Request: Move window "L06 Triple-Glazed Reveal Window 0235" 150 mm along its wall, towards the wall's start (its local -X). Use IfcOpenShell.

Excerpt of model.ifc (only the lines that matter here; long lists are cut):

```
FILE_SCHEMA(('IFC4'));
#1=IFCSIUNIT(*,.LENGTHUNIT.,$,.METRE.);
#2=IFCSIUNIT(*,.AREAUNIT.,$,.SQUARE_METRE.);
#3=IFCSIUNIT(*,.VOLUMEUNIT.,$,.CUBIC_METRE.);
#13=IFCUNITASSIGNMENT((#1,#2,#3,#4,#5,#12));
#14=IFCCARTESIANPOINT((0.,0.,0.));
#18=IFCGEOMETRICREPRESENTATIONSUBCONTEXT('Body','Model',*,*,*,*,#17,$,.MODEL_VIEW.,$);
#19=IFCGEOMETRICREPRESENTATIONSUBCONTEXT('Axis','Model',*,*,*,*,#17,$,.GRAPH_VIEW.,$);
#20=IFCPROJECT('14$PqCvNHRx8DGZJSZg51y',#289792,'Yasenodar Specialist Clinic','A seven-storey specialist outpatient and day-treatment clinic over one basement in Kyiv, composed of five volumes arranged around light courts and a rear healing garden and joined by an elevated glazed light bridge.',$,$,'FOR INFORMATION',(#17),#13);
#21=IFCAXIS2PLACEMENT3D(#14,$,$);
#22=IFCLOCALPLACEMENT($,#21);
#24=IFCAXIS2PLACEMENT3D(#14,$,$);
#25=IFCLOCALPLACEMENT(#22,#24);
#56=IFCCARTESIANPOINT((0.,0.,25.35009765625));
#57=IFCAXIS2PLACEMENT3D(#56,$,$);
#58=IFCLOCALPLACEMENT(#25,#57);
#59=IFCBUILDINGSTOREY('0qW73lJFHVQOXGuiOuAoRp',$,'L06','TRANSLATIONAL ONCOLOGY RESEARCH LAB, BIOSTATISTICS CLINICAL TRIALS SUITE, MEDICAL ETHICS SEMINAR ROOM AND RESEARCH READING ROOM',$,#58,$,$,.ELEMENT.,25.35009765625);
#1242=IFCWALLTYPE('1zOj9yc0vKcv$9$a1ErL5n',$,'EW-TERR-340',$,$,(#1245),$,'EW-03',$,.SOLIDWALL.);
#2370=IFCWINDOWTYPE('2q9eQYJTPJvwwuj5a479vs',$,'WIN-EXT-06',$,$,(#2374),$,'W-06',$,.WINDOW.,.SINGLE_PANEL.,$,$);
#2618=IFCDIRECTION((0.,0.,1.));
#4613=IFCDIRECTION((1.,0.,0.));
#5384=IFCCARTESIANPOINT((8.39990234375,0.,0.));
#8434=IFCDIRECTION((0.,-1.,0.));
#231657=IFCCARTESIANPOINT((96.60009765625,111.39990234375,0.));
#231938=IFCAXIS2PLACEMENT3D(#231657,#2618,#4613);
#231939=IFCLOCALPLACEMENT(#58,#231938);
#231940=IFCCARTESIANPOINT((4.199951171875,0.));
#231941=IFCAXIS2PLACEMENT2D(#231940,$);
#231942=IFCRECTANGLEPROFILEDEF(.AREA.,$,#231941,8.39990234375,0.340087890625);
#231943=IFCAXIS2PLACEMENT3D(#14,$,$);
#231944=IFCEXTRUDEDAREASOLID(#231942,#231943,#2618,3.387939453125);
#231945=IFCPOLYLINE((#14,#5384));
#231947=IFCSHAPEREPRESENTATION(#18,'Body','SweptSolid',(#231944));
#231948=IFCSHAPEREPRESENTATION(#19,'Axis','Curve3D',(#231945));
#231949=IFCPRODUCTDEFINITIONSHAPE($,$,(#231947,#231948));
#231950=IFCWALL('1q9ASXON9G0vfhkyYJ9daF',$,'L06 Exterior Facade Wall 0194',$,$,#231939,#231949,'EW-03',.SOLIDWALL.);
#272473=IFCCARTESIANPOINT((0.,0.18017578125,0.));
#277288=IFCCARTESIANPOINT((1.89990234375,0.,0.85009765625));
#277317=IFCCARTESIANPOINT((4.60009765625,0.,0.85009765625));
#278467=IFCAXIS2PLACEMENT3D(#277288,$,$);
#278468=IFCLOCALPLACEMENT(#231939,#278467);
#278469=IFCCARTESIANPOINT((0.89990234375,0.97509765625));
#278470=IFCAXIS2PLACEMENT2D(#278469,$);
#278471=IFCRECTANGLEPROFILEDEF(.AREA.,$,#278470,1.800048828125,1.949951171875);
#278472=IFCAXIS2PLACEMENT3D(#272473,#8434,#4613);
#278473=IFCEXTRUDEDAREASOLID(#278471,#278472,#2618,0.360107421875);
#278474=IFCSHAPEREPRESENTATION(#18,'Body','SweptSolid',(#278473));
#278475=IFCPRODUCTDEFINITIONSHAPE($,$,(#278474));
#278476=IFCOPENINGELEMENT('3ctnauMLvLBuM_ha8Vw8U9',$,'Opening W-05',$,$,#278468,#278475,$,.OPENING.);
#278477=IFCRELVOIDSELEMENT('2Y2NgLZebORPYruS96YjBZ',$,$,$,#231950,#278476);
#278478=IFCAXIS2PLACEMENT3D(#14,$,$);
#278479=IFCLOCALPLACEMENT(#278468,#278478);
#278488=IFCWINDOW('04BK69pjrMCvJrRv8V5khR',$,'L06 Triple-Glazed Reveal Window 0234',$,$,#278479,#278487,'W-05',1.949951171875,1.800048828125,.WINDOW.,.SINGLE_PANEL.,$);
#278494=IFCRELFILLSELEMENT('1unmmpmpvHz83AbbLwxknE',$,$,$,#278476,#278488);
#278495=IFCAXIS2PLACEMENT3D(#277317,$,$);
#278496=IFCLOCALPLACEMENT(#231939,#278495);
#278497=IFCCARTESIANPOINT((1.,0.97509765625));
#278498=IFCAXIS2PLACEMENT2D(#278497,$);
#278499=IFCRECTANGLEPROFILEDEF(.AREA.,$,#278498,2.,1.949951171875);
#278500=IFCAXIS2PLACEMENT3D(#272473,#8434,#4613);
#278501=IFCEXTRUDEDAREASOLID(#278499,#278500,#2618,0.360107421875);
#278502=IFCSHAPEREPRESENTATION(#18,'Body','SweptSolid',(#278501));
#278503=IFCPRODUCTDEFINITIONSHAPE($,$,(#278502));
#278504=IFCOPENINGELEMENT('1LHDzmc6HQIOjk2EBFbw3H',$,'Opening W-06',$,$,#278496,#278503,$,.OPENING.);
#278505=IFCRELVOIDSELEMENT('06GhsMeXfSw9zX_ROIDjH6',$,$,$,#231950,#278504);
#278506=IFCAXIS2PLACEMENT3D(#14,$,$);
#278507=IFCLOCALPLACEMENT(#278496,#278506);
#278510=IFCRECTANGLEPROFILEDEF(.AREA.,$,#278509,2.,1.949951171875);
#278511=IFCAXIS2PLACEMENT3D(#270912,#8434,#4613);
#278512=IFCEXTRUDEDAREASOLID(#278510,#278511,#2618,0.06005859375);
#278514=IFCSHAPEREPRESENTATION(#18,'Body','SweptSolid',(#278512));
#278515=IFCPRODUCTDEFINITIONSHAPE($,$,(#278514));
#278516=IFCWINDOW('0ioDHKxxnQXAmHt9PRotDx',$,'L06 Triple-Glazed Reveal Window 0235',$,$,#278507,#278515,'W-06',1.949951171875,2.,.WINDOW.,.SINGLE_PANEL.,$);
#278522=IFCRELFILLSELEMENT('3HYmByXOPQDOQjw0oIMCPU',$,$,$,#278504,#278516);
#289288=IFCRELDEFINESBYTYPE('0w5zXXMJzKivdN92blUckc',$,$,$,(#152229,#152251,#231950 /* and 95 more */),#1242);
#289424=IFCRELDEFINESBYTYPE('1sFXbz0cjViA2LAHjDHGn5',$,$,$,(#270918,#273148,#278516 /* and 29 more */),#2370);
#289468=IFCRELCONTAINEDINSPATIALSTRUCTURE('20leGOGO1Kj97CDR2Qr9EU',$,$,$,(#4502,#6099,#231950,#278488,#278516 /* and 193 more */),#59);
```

```python
import ifcopenshell
import ifcopenshell.api.geometry
import ifcopenshell.util.placement

model = ifcopenshell.open("model.ifc")

window = model.by_id(278516)
opening = window.FillsVoids[0].RelatingOpeningElement
wall = opening.VoidsElements[0].RelatingBuildingElement

wall_matrix = ifcopenshell.util.placement.get_local_placement(wall.ObjectPlacement)
shift = wall_matrix[:3, 0] * -0.15
before = ifcopenshell.util.placement.get_local_placement(window.ObjectPlacement)[:3, 3].copy()

# The window is placed relative to its opening, so it follows when the opening moves.
matrix = ifcopenshell.util.placement.get_local_placement(opening.ObjectPlacement)
matrix[:3, 3] += shift
ifcopenshell.api.geometry.edit_object_placement(
    model, product=opening, matrix=matrix, is_si=False, should_transform_children=True
)

after = ifcopenshell.util.placement.get_local_placement(window.ObjectPlacement)[:3, 3]
print("window moved by", (after - before).round(3) + 0.0)

model.write("model_v2.ifc")
```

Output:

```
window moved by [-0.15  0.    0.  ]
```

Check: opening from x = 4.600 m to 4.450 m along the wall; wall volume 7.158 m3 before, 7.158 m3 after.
